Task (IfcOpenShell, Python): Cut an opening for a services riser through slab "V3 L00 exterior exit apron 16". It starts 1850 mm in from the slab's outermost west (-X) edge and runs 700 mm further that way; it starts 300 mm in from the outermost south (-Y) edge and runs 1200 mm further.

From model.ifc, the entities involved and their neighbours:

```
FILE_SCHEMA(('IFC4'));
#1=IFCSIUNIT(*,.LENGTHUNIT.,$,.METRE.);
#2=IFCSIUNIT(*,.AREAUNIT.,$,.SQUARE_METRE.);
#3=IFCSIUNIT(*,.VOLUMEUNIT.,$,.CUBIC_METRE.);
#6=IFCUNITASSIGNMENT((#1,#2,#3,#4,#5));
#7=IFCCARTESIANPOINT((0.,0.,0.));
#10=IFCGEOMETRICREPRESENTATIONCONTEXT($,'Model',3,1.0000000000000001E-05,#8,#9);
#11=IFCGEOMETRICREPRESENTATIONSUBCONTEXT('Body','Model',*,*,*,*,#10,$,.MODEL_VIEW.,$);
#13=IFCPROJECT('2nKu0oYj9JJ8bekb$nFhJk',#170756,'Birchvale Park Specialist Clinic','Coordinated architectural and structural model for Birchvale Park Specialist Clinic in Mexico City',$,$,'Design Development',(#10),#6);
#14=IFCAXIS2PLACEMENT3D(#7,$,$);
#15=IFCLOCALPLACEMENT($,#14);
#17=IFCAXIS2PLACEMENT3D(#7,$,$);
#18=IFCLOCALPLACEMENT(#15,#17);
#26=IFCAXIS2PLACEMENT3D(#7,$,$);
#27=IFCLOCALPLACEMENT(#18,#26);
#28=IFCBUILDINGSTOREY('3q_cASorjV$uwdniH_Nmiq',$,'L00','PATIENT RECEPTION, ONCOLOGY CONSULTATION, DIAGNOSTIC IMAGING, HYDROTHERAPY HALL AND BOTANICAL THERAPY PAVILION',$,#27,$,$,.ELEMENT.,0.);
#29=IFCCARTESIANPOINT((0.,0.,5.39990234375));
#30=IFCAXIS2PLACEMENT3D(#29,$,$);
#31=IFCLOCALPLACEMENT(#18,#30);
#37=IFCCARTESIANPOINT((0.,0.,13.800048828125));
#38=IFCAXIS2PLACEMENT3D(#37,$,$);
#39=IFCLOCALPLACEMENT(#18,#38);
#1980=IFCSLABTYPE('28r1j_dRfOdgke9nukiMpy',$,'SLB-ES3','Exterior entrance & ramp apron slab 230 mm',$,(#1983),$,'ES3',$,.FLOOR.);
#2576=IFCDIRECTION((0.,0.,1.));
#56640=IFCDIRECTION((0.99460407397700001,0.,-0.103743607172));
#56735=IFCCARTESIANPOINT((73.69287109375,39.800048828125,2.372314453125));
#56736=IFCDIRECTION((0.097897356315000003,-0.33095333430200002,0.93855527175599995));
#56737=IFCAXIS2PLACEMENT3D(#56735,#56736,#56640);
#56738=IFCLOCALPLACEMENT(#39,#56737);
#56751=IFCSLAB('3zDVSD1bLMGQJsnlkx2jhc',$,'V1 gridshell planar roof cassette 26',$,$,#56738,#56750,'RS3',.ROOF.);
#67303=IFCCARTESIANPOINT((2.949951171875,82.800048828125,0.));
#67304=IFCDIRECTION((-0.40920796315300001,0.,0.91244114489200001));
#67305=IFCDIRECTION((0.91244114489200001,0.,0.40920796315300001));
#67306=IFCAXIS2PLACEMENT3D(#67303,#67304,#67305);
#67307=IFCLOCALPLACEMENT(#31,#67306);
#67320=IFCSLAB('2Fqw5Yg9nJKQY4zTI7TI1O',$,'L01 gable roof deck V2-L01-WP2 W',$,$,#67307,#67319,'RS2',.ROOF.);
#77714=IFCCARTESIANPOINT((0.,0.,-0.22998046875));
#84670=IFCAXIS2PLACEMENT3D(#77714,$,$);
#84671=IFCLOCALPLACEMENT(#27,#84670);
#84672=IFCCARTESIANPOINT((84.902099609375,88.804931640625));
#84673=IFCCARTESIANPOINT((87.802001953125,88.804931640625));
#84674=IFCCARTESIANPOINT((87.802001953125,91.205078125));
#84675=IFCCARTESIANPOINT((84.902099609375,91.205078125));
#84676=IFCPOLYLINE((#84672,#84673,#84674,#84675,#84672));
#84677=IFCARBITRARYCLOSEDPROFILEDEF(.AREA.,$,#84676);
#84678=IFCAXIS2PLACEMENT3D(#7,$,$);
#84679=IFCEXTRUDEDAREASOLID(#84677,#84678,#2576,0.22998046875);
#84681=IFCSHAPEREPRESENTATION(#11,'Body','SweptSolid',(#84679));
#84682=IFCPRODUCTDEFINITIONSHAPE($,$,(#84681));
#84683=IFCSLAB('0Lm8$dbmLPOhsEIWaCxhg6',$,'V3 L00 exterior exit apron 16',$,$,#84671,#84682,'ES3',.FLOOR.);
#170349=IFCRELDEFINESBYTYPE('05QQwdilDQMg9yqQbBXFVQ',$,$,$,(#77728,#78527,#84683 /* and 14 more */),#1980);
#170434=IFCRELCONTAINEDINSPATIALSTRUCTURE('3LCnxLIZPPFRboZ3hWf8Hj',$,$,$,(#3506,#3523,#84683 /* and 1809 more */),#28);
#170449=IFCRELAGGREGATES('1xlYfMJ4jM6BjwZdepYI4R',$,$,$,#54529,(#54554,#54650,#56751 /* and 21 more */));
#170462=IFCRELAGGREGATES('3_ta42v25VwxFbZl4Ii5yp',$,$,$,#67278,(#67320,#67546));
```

```python
import numpy as np
import ifcopenshell
import ifcopenshell.api.feature
import ifcopenshell.api.geometry
import ifcopenshell.api.root
import ifcopenshell.geom
import ifcopenshell.util.placement
import ifcopenshell.util.representation
import ifcopenshell.util.shape
import ifcopenshell.util.unit

model = ifcopenshell.open("model.ifc")
unit_scale = ifcopenshell.util.unit.calculate_unit_scale(model)
settings = ifcopenshell.geom.settings()


def volume(element):
    """Net volume in cubic metres, openings subtracted."""
    shape = ifcopenshell.geom.create_shape(settings, element)
    return ifcopenshell.util.shape.get_volume(shape.geometry)


slab = model.by_guid("0Lm8$dbmLPOhsEIWaCxhg6")
before = volume(slab)

# Extent in the slab's own axes, in metres. The edges named are its -X and -Y sides.
slab_shape = ifcopenshell.geom.create_shape(settings, slab)
vertices = ifcopenshell.util.shape.get_vertices(slab_shape.geometry)
x_min, y_min, bottom = vertices.min(axis=0)
top = vertices[:, 2].max()

opening = ifcopenshell.api.root.create_entity(model, ifc_class="IfcOpeningElement", name="Services riser opening", predefined_type="OPENING")
context = ifcopenshell.util.representation.get_context(model, "Model", "Body", "MODEL_VIEW")
width, depth = 0.7, 1.2
outline = [(0.0, 0.0), (width, 0.0), (width, depth), (0.0, depth), (0.0, 0.0)]
# Overshoot both faces by 50 mm so the cut is clean.
shape = ifcopenshell.api.geometry.add_slab_representation(
    model, context=context, depth=top - bottom + 0.1, polyline=outline
)
ifcopenshell.api.geometry.assign_representation(model, product=opening, representation=shape)

matrix = ifcopenshell.util.placement.get_local_placement(slab.ObjectPlacement)
matrix[:, 3] = matrix @ np.append(np.array([x_min + 1.85, y_min + 0.3, bottom - 0.05]) / unit_scale, 1.0)
ifcopenshell.api.geometry.edit_object_placement(model, product=opening, matrix=matrix, is_si=False)
ifcopenshell.api.feature.add_feature(model, feature=opening, element=slab)

after = volume(slab)

print(f"slab volume {before:.3f} -> {after:.3f} m3")

model.write("model_rev.ifc")
```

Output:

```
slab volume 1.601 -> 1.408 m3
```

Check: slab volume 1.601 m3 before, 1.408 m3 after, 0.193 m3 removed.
